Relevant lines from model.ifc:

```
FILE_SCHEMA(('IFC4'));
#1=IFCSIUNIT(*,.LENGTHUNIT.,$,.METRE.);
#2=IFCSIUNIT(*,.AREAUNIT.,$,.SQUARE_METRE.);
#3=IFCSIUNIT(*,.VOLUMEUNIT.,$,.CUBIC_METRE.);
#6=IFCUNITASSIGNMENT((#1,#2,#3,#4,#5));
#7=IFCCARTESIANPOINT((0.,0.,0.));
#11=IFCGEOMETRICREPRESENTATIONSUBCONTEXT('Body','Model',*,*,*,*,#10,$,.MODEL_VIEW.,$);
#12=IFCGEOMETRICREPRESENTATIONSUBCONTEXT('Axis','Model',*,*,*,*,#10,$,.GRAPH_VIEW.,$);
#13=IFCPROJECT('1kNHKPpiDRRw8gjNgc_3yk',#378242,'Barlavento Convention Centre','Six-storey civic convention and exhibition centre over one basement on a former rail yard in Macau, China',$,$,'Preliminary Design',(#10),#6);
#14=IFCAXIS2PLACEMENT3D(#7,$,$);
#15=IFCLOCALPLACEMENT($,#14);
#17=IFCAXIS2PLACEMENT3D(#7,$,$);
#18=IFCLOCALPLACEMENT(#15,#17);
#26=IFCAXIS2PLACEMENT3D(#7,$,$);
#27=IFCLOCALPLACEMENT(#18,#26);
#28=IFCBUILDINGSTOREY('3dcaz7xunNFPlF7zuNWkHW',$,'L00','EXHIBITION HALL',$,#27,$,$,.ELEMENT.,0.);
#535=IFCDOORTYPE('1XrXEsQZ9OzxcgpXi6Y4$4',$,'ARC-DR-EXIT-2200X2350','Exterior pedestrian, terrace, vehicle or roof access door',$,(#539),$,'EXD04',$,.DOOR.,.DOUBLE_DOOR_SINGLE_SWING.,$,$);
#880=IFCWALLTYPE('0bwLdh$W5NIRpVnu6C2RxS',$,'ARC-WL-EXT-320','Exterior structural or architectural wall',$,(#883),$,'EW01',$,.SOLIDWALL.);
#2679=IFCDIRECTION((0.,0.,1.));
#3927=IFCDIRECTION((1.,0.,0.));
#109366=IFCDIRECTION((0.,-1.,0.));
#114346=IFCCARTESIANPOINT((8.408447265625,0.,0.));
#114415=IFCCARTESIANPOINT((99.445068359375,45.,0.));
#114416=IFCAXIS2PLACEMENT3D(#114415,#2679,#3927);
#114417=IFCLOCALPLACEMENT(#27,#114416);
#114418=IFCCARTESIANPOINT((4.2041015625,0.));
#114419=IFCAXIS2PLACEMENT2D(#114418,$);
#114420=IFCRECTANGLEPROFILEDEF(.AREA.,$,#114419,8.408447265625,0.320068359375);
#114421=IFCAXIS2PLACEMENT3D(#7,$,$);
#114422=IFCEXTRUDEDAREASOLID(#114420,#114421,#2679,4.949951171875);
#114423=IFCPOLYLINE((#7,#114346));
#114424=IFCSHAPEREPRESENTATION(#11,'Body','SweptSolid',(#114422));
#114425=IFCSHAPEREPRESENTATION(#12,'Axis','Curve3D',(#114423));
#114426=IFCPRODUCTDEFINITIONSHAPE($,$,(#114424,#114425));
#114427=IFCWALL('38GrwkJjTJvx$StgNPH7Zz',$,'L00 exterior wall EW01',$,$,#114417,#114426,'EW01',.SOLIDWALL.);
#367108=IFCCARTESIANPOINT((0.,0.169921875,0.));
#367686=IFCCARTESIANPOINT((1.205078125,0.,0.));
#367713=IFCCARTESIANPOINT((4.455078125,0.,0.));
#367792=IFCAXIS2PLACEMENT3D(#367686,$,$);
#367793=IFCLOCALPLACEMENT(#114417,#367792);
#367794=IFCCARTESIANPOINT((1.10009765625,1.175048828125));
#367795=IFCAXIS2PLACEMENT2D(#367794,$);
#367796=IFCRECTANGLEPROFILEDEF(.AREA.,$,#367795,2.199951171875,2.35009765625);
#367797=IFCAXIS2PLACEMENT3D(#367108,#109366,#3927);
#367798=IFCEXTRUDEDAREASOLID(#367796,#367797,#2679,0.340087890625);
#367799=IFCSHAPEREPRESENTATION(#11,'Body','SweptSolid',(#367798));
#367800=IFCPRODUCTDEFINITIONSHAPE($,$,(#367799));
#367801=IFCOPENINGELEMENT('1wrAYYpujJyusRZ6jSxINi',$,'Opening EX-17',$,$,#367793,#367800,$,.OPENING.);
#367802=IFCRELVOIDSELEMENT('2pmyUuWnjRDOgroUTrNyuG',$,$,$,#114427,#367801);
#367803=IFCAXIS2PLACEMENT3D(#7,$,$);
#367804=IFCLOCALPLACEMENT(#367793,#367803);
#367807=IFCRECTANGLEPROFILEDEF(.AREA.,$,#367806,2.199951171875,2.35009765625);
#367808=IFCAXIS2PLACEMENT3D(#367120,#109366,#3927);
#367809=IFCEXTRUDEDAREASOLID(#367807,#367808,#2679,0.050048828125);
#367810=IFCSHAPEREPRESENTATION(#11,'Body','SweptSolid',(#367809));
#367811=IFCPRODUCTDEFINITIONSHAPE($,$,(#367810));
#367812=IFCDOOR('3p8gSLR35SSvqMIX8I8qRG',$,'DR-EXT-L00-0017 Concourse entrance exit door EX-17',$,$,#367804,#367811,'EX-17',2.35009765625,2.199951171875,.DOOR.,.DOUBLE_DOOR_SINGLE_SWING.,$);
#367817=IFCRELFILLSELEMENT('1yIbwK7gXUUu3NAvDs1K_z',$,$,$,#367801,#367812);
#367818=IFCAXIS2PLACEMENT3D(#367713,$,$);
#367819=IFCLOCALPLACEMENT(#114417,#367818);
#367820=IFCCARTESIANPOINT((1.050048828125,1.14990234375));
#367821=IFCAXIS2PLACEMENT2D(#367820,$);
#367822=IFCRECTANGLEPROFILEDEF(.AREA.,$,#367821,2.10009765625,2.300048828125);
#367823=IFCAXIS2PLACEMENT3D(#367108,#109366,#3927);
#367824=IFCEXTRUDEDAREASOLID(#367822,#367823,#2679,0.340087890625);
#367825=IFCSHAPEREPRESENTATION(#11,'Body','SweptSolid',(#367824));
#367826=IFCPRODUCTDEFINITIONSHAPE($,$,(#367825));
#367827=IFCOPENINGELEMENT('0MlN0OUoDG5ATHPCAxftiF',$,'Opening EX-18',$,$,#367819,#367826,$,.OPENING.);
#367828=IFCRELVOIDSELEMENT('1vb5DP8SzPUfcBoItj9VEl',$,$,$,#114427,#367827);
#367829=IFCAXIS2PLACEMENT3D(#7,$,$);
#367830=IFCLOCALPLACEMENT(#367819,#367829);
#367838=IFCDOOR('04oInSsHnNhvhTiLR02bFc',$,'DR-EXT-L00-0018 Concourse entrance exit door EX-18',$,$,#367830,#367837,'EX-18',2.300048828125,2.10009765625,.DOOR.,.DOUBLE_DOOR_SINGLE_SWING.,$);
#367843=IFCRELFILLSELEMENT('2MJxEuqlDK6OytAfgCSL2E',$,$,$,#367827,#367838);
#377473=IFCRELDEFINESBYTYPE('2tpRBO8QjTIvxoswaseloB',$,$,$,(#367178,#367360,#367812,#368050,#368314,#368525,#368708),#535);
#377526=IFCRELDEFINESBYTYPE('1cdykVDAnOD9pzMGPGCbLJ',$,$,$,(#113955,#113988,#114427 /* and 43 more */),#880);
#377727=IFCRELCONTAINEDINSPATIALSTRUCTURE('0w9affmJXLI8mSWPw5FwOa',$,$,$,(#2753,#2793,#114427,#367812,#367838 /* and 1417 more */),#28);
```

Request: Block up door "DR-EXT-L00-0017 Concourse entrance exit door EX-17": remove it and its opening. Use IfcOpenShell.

```python
import ifcopenshell
import ifcopenshell.api.feature
import ifcopenshell.api.root
import ifcopenshell.geom
import ifcopenshell.util.shape

model = ifcopenshell.open("model.ifc")
settings = ifcopenshell.geom.settings()


def volume(element):
    """Net volume in cubic metres, openings subtracted."""
    shape = ifcopenshell.geom.create_shape(settings, element)
    return ifcopenshell.util.shape.get_volume(shape.geometry)


door = model.by_guid("3p8gSLR35SSvqMIX8I8qRG")
opening = door.FillsVoids[0].RelatingOpeningElement
wall = opening.VoidsElements[0].RelatingBuildingElement
before = volume(wall)

ifcopenshell.api.root.remove_product(model, product=door)
ifcopenshell.api.feature.remove_feature(model, feature=opening)

after = volume(wall)

print(f"wall volume {before:.3f} -> {after:.3f} m3")

model.write("model_rev.ifc")
```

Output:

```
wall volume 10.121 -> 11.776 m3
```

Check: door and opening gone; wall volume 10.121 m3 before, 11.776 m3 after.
